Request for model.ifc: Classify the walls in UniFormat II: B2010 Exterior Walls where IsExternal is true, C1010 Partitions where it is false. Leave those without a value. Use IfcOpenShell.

First a look at what the model holds.

```python
import ifcopenshell
import ifcopenshell.util.element

model = ifcopenshell.open("model.ifc")
print(model.schema)
print("classifications:", [c.Name for c in model.by_type("IfcClassification")])
values = [ifcopenshell.util.element.get_pset(e, "Pset_WallCommon", "IsExternal") for e in model.by_type("IfcWall")]
for value in (True, False, None):
    print("IsExternal", value, values.count(value))
```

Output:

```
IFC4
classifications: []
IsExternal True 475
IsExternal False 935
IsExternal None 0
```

```python
import ifcopenshell
import ifcopenshell.api.classification
import ifcopenshell.util.element

model = ifcopenshell.open("model.ifc")

system = ifcopenshell.api.classification.add_classification(model, classification="UniFormat II")

walls = model.by_type("IfcWall")
external = {e: ifcopenshell.util.element.get_pset(e, "Pset_WallCommon", "IsExternal") for e in walls}
for flag, code, name in ((True, "B2010", "Exterior Walls"), (False, "C1010", "Partitions")):
    products = [e for e in walls if external[e] is flag]
    ifcopenshell.api.classification.add_reference(
        model, products=products, classification=system, identification=code, name=name
    )
    print(code, len(products))

model.write("model_updated.ifc")
```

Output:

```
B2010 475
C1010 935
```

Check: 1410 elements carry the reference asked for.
